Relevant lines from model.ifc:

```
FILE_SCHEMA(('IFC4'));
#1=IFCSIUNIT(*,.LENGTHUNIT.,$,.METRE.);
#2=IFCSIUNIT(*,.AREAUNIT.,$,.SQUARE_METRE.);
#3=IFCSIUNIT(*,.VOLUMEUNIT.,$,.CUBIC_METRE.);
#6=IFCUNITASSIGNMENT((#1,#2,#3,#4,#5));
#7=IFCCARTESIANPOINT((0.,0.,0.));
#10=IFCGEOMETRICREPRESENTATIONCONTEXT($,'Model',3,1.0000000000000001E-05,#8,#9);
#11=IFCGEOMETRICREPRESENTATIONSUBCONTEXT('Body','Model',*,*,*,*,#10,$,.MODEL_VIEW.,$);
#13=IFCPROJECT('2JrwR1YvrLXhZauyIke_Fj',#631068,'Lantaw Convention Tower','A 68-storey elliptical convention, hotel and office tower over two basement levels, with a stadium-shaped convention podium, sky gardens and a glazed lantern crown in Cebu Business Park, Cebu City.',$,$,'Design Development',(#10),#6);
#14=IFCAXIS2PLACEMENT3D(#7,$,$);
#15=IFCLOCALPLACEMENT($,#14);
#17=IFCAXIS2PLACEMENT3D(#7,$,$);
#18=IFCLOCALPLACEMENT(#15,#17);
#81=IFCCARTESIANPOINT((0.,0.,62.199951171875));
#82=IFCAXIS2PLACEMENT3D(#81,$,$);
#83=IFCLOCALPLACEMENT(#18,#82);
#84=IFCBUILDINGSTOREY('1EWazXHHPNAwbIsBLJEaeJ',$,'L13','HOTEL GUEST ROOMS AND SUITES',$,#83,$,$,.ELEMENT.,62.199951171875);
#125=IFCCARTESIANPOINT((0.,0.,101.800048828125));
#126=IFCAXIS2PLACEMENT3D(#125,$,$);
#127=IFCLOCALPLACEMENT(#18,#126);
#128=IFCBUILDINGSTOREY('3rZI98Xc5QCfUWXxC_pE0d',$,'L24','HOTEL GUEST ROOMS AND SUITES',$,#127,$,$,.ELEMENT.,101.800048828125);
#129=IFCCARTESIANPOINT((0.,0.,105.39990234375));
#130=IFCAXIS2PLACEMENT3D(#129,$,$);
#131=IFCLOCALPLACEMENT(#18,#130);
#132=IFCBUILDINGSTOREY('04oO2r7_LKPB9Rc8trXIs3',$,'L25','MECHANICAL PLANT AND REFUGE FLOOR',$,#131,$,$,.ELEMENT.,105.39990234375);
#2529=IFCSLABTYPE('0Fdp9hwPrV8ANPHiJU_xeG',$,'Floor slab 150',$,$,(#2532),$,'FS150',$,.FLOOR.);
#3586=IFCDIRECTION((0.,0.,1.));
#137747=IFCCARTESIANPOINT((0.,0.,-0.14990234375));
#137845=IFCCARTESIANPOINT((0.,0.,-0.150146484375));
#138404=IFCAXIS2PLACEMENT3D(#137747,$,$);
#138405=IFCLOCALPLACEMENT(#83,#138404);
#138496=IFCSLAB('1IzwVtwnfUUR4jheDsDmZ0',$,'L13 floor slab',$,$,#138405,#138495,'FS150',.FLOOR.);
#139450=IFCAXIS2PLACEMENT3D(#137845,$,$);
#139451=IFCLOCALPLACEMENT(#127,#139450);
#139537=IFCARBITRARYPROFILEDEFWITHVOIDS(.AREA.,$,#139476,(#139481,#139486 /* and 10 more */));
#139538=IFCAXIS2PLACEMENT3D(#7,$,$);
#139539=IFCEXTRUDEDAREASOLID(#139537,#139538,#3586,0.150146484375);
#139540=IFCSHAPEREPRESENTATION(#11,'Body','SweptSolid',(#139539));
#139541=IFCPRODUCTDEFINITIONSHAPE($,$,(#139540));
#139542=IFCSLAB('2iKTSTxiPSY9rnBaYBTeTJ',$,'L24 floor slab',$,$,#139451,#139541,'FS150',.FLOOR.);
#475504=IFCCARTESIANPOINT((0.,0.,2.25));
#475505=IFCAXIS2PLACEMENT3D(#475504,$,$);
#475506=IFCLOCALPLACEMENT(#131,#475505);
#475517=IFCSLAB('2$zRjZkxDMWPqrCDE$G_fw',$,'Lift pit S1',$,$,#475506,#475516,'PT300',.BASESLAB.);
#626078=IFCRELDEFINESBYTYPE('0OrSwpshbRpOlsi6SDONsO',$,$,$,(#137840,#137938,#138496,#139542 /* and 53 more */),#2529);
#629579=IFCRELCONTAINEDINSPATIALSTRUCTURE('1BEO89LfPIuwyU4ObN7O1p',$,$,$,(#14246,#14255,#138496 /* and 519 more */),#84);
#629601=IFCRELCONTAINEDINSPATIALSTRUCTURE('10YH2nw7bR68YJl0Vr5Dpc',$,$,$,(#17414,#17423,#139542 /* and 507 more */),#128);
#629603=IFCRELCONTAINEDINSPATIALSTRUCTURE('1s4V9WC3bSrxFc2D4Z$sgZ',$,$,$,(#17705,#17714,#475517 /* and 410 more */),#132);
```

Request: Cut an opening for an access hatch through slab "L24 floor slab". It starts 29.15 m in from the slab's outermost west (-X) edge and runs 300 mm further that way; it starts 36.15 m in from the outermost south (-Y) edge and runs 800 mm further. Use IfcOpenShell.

```python
import numpy as np
import ifcopenshell
import ifcopenshell.api.feature
import ifcopenshell.api.geometry
import ifcopenshell.api.root
import ifcopenshell.geom
import ifcopenshell.util.placement
import ifcopenshell.util.representation
import ifcopenshell.util.shape
import ifcopenshell.util.unit

model = ifcopenshell.open("model.ifc")
unit_scale = ifcopenshell.util.unit.calculate_unit_scale(model)
settings = ifcopenshell.geom.settings()


def volume(element):
    """Net volume in cubic metres, openings subtracted."""
    shape = ifcopenshell.geom.create_shape(settings, element)
    return ifcopenshell.util.shape.get_volume(shape.geometry)


slab = model.by_guid("2iKTSTxiPSY9rnBaYBTeTJ")
before = volume(slab)

# Extent in the slab's own axes, in metres. The edges named are its -X and -Y sides.
slab_shape = ifcopenshell.geom.create_shape(settings, slab)
vertices = ifcopenshell.util.shape.get_vertices(slab_shape.geometry)
x_min, y_min, bottom = vertices.min(axis=0)
top = vertices[:, 2].max()

opening = ifcopenshell.api.root.create_entity(model, ifc_class="IfcOpeningElement", name="Access hatch opening", predefined_type="OPENING")
context = ifcopenshell.util.representation.get_context(model, "Model", "Body", "MODEL_VIEW")
width, depth = 0.3, 0.8
outline = [(0.0, 0.0), (width, 0.0), (width, depth), (0.0, depth), (0.0, 0.0)]
# Overshoot both faces by 50 mm so the cut is clean.
shape = ifcopenshell.api.geometry.add_slab_representation(
    model, context=context, depth=top - bottom + 0.1, polyline=outline
)
ifcopenshell.api.geometry.assign_representation(model, product=opening, representation=shape)

matrix = ifcopenshell.util.placement.get_local_placement(slab.ObjectPlacement)
matrix[:, 3] = matrix @ np.append(np.array([x_min + 29.15, y_min + 36.15, bottom - 0.05]) / unit_scale, 1.0)
ifcopenshell.api.geometry.edit_object_placement(model, product=opening, matrix=matrix, is_si=False)
ifcopenshell.api.feature.add_feature(model, feature=opening, element=slab)

after = volume(slab)

print(f"slab volume {before:.3f} -> {after:.3f} m3")

model.write("model_rev.ifc")
```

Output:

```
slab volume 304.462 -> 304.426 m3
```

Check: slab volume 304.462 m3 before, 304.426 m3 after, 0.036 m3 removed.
